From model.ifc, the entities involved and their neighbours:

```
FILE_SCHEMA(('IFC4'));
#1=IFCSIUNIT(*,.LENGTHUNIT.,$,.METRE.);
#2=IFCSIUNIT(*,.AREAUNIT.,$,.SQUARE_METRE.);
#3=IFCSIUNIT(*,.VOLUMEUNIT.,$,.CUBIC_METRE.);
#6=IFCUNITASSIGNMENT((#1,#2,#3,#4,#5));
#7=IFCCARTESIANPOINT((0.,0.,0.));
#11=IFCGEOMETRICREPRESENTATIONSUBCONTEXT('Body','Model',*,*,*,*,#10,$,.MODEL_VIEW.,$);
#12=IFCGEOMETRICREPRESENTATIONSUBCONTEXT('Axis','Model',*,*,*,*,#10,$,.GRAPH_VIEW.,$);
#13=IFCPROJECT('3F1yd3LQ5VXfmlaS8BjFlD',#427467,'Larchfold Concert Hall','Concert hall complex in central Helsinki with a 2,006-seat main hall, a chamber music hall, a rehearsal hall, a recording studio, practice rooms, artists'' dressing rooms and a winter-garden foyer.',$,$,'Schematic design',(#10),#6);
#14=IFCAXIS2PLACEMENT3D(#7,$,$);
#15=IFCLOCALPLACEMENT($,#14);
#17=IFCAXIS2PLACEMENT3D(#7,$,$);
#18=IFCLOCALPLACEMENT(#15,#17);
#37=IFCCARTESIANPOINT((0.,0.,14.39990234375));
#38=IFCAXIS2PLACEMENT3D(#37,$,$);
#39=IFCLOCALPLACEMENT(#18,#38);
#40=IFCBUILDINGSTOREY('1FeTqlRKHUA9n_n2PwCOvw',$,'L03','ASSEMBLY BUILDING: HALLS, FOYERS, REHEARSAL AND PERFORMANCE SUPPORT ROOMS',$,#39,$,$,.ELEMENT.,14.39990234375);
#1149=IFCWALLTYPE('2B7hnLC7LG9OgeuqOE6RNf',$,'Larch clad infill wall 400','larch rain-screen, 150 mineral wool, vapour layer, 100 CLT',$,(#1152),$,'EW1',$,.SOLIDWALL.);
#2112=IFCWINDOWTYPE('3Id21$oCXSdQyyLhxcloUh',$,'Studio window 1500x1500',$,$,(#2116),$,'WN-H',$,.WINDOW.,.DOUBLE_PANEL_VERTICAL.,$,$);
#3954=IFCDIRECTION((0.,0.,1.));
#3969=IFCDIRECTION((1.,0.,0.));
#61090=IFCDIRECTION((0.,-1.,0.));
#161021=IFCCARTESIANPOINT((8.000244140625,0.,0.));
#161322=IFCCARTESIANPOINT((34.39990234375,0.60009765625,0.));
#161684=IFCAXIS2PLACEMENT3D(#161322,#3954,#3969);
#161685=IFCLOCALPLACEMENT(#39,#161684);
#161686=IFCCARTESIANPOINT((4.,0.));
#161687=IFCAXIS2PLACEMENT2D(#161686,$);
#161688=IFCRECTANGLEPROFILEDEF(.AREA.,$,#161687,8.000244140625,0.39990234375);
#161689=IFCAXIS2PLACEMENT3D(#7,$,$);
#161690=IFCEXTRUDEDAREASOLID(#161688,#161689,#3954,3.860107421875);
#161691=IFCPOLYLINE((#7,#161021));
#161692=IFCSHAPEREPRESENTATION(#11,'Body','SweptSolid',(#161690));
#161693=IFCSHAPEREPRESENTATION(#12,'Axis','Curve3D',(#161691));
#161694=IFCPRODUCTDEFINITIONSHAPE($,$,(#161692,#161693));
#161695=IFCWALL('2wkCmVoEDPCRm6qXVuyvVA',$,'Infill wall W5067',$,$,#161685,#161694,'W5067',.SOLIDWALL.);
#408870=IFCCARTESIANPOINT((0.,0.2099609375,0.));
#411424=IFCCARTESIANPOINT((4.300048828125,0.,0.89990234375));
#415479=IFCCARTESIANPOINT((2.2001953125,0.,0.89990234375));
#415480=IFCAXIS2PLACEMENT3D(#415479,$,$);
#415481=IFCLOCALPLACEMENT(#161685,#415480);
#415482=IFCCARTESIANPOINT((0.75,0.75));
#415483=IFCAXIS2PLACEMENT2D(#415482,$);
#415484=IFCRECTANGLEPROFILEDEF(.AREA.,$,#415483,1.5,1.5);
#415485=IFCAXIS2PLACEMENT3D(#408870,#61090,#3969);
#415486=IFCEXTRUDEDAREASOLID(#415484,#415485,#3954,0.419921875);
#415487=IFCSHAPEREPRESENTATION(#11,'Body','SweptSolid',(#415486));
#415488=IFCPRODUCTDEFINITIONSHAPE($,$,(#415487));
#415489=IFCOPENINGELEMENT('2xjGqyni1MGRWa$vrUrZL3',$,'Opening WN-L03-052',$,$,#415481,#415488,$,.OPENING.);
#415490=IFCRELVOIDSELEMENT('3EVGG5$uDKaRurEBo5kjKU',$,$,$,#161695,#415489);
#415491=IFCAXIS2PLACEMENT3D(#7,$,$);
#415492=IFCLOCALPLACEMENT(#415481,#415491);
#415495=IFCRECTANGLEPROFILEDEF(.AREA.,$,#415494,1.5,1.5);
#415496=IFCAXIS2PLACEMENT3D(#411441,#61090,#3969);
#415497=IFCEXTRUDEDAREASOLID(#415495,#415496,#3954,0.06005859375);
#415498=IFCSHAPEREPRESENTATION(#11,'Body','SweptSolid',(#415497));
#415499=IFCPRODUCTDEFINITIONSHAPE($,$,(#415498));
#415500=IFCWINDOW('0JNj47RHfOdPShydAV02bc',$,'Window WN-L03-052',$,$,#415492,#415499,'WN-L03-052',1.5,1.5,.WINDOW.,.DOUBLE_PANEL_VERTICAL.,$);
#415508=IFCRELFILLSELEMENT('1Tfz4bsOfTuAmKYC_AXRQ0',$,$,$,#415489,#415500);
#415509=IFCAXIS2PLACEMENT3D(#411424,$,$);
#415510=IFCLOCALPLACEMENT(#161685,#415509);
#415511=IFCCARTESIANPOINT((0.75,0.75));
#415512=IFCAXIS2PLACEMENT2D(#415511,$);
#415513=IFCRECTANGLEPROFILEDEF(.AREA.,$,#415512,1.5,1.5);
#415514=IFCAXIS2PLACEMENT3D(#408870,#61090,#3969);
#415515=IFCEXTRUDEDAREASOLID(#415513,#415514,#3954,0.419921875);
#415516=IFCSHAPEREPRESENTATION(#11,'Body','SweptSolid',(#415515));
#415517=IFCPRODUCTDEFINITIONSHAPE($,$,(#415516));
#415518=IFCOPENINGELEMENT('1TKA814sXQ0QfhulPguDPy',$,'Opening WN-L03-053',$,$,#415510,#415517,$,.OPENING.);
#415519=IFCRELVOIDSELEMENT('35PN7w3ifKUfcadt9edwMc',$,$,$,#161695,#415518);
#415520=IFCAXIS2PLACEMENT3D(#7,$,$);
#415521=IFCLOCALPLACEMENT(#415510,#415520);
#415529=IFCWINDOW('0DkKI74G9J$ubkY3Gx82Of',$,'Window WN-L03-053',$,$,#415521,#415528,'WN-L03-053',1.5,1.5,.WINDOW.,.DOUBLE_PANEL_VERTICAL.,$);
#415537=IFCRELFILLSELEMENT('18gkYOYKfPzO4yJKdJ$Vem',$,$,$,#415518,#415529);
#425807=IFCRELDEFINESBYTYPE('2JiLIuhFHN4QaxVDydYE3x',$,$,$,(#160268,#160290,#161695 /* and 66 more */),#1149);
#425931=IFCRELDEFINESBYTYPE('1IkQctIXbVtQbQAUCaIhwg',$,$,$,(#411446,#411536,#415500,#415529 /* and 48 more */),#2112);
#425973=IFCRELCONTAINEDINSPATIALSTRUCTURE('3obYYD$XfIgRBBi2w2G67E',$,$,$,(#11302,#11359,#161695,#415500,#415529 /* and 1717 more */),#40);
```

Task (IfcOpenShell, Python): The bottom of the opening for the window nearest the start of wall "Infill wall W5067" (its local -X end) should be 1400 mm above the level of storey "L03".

```python
import numpy as np
import ifcopenshell
import ifcopenshell.api.geometry
import ifcopenshell.geom
import ifcopenshell.util.element
import ifcopenshell.util.placement
import ifcopenshell.util.shape
import ifcopenshell.util.unit

model = ifcopenshell.open("model.ifc")
unit_scale = ifcopenshell.util.unit.calculate_unit_scale(model)

window = model.by_guid("0JNj47RHfOdPShydAV02bc")
opening = window.FillsVoids[0].RelatingOpeningElement
storey = ifcopenshell.util.element.get_container(window, ifc_class="IfcBuildingStorey")
level = ifcopenshell.util.placement.get_local_placement(storey.ObjectPlacement)[2, 3]

# The opening's origin need not be at the sill, so measure its lowest point.
shape = ifcopenshell.geom.create_shape(ifcopenshell.geom.settings(), opening)
bottom = ifcopenshell.util.shape.get_shape_bottom_elevation(shape, shape.geometry) / unit_scale
dz = level + 1.4 / unit_scale - bottom

shift = np.array([0.0, 0.0, dz])
# The window is placed relative to its opening, so it follows when the opening moves.
matrix = ifcopenshell.util.placement.get_local_placement(opening.ObjectPlacement)
matrix[:3, 3] += shift
ifcopenshell.api.geometry.edit_object_placement(
    model, product=opening, matrix=matrix, is_si=False, should_transform_children=True
)

print(f"moved by {dz * unit_scale:+.3f} m")

model.write("model_updated.ifc")
```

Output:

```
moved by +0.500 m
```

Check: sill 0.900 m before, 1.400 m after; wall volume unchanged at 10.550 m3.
